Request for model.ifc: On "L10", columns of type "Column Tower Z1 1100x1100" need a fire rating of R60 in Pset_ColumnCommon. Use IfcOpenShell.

First a look at what the model holds.

```python
import ifcopenshell
import ifcopenshell.util.element

model = ifcopenshell.open("model.ifc")
print(model.schema)
storey = next(s for s in model.by_type("IfcBuildingStorey") if s.Name == "L10")
columns = [e for e in ifcopenshell.util.element.get_decomposition(storey) if e.is_a("IfcColumn")]
seen = {}
for e in columns:
    element_type = ifcopenshell.util.element.get_type(e)
    key = (element_type.Name if element_type != e and element_type else None, ifcopenshell.util.element.get_pset(e, "Pset_ColumnCommon", "FireRating"))
    seen[key] = seen.get(key, 0) + 1
for (name, value), count in sorted(seen.items(), key=str):
    print(count, "x", name, "|", value)
```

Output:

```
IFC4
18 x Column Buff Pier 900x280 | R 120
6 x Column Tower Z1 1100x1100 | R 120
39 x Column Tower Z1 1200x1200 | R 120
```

```python
import ifcopenshell
import ifcopenshell.api.pset
import ifcopenshell.util.element

model = ifcopenshell.open("model.ifc")

storey = next(s for s in model.by_type("IfcBuildingStorey") if s.Name == "L10")
columns = [e for e in ifcopenshell.util.element.get_decomposition(storey) if e.is_a("IfcColumn")]

count = 0
for e in columns:
    element_type = ifcopenshell.util.element.get_type(e)
    if element_type in (None, e) or element_type.Name != "Column Tower Z1 1100x1100":
        continue
    found = ifcopenshell.util.element.get_pset(e, "Pset_ColumnCommon", should_inherit=False)
    if found:
        pset = model.by_id(found["id"])
        if len(ifcopenshell.util.element.get_elements_by_pset(pset)) > 1:
            pset = ifcopenshell.api.pset.unshare_pset(model, products=[e], pset=pset)[0]
    else:
        pset = ifcopenshell.api.pset.add_pset(model, product=e, name="Pset_ColumnCommon")
    ifcopenshell.api.pset.edit_pset(model, pset=pset, properties={"FireRating": "R60"})
    count += 1

print(count, "columns updated")

model.write("model_rev.ifc")
```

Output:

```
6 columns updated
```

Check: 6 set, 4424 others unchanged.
